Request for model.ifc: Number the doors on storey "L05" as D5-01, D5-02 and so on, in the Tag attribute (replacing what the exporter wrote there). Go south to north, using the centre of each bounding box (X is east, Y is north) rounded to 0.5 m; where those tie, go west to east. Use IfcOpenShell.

First a look at what the model holds.

```python
import ifcopenshell
import ifcopenshell.util.element
import ifcopenshell.util.placement

model = ifcopenshell.open("model.ifc")
print(model.schema)
storey = next(s for s in model.by_type("IfcBuildingStorey") if s.Name == "L05")
doors = [e for e in ifcopenshell.util.element.get_decomposition(storey) if e.is_a("IfcDoor")]
for e in sorted(doors, key=lambda e: e.id()):
    origin = ifcopenshell.util.placement.get_local_placement(e.ObjectPlacement)[:3, 3]
    print(e.id(), e.Tag, e.Name, origin.round(2) + 0.0, sep=" | ")
```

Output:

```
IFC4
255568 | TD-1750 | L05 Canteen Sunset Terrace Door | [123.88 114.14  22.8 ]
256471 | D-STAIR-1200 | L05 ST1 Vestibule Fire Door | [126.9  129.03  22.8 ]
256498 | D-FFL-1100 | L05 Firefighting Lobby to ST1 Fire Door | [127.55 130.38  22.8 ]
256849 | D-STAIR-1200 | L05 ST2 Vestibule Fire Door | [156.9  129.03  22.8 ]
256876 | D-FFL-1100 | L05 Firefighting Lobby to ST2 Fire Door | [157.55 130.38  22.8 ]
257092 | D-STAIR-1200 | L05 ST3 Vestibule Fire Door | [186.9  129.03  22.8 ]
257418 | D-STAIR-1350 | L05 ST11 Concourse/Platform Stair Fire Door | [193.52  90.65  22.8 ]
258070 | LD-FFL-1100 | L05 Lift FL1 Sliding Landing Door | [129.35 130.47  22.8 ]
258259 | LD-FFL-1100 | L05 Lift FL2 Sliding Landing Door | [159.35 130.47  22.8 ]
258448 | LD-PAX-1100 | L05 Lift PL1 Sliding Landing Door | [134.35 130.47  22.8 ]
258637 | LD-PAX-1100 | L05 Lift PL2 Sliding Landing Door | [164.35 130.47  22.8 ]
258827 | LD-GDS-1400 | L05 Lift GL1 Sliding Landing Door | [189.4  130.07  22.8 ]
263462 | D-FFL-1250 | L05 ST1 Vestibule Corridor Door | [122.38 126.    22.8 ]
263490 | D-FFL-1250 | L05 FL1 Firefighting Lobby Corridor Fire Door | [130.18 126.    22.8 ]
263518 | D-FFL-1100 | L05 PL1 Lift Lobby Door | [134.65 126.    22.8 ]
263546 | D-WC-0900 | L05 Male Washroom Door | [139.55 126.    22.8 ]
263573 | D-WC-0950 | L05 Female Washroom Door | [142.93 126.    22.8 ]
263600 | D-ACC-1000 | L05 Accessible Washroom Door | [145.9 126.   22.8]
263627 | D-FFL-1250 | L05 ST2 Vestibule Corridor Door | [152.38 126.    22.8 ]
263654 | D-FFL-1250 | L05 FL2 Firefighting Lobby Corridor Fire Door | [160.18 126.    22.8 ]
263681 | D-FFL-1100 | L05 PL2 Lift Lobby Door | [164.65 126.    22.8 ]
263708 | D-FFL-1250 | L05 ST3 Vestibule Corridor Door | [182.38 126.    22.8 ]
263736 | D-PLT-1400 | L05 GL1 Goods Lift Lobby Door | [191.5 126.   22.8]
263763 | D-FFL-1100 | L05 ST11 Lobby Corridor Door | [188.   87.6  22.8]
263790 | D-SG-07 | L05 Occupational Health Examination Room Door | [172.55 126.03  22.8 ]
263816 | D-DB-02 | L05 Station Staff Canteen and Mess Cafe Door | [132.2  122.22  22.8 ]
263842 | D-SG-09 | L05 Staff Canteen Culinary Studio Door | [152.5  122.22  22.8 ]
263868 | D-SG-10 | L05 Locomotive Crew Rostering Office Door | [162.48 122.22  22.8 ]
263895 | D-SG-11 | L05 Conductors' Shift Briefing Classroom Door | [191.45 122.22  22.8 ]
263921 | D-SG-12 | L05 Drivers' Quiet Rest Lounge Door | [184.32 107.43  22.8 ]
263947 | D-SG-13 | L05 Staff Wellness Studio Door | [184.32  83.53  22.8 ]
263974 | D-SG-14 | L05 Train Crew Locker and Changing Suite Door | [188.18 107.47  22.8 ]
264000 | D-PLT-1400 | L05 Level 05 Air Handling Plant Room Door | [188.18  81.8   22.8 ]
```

```python
import ifcopenshell
import ifcopenshell.geom
import ifcopenshell.util.element
import ifcopenshell.util.shape

model = ifcopenshell.open("model.ifc")
settings = ifcopenshell.geom.settings()
settings.set("use-world-coords", True)


def centre(element):
    shape = ifcopenshell.geom.create_shape(settings, element)
    return ifcopenshell.util.shape.get_bbox_centroid(shape.geometry)


storey = next(s for s in model.by_type("IfcBuildingStorey") if s.Name == "L05")
doors = [e for e in ifcopenshell.util.element.get_decomposition(storey) if e.is_a("IfcDoor")]

# Insertion points can sit at a corner or the storey origin, so sort by the geometry (in metres).
centres = {e: centre(e) for e in doors}
doors.sort(key=lambda e: (round(centres[e][1] / 0.5), centres[e][0]))

for i, e in enumerate(doors, start=1):
    number = f"D5-{i:02d}"
    e.Tag = number
    print(e.id(), number)

model.write("model_v2.ifc")
```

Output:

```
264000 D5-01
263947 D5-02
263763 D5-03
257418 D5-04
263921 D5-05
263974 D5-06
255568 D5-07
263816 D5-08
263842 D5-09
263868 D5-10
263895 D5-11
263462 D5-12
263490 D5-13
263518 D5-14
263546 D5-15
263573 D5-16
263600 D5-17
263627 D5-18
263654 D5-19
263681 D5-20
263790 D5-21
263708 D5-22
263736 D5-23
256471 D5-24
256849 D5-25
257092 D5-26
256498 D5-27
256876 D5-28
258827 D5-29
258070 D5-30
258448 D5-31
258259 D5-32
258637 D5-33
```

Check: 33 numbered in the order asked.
